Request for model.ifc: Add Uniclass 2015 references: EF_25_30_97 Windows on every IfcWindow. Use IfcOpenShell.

First a look at what the model holds.

```python
import ifcopenshell

model = ifcopenshell.open("model.ifc")
print(model.schema)
print("classifications:", [c.Name for c in model.by_type("IfcClassification")])
for ifc_class in ("IfcDoor", "IfcRoof", "IfcStair", "IfcWall", "IfcWindow"):
    print(ifc_class, len(model.by_type(ifc_class)))
```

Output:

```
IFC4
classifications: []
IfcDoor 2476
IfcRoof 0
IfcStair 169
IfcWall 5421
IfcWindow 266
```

```python
import ifcopenshell
import ifcopenshell.api.classification

model = ifcopenshell.open("model.ifc")

system = ifcopenshell.api.classification.add_classification(model, classification="Uniclass 2015")

codes = {
    "IfcWindow": ("EF_25_30_97", "Windows"),
}
for ifc_class, (code, name) in codes.items():
    products = model.by_type(ifc_class)
    ifcopenshell.api.classification.add_reference(
        model, products=products, classification=system, identification=code, name=name
    )
    print(code, len(products))

model.write("model_v2.ifc")
```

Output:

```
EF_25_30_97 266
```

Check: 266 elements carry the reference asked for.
